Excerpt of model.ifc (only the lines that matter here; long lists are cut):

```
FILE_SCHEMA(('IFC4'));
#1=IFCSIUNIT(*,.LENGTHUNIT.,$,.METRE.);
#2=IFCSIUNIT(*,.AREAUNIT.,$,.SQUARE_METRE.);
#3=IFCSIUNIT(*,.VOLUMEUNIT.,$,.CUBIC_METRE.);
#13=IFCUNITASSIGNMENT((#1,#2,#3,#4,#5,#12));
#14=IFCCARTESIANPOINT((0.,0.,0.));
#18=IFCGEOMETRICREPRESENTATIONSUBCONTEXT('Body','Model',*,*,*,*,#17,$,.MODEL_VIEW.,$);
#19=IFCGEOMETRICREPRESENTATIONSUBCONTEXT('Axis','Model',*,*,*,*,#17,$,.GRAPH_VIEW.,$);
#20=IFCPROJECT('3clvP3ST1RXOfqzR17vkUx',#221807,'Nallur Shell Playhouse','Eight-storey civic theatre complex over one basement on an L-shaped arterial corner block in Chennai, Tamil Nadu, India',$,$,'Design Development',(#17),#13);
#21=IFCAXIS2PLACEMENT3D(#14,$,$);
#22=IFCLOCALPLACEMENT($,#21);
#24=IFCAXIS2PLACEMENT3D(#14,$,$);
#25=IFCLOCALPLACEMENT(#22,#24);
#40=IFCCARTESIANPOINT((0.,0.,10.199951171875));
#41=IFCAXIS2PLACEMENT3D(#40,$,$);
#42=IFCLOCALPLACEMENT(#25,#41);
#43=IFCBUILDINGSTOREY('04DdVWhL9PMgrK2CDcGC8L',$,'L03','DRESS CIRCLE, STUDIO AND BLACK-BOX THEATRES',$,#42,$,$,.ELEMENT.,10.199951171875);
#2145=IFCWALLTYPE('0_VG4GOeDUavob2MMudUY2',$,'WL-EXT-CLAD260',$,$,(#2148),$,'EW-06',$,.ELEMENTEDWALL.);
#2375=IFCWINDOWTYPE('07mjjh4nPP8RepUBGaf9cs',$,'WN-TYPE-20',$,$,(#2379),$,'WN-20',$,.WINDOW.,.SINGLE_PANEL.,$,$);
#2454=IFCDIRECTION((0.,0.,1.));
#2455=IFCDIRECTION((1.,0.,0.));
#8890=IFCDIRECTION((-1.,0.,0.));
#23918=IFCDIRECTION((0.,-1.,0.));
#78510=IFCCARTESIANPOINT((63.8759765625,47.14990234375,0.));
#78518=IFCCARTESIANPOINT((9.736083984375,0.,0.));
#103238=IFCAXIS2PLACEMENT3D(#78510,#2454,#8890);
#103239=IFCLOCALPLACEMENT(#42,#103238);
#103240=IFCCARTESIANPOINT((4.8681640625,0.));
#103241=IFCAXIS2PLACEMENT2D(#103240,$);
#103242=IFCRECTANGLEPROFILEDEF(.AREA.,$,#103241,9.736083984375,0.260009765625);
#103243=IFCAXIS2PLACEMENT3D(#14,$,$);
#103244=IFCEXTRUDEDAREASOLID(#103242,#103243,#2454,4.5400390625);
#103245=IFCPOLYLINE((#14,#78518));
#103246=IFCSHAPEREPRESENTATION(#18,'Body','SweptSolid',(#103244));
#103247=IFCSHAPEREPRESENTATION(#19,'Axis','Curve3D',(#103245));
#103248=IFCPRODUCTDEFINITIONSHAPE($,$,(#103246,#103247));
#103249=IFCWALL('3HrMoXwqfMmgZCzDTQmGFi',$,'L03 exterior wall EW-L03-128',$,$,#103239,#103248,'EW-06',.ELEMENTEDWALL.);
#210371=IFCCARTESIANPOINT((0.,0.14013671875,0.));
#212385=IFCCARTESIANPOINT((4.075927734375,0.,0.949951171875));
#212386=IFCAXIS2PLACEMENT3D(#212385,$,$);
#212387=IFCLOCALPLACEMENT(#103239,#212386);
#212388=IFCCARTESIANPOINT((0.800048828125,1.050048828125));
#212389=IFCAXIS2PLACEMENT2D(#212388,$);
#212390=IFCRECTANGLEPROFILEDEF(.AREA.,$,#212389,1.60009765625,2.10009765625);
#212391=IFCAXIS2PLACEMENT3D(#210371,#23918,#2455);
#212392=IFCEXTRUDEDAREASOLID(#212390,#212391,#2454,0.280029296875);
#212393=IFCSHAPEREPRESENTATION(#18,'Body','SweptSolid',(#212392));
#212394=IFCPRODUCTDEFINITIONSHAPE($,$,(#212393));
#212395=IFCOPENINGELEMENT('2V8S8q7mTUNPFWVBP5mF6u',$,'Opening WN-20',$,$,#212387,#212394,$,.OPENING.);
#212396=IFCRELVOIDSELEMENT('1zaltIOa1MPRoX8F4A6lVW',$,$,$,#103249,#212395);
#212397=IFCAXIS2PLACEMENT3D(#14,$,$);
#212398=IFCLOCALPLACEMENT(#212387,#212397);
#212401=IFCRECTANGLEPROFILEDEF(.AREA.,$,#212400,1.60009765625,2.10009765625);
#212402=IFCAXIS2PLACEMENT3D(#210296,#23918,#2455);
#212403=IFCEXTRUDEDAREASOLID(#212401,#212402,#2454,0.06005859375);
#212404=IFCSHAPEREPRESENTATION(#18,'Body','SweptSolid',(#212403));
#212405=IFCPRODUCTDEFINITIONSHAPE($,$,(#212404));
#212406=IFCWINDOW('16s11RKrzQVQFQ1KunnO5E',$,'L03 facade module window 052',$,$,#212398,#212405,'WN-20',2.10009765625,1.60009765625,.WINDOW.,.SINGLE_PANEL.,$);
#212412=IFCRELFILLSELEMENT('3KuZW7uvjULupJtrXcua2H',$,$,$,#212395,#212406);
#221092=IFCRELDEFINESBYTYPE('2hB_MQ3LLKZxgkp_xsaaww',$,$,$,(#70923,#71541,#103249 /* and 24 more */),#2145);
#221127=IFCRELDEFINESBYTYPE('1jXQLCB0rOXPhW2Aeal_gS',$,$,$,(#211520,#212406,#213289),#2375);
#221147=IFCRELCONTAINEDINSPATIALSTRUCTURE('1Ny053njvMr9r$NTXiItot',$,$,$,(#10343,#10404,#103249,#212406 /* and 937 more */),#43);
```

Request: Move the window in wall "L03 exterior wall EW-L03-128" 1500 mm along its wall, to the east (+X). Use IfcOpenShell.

```python
import ifcopenshell
import ifcopenshell.api.geometry
import ifcopenshell.util.placement
import ifcopenshell.util.unit

model = ifcopenshell.open("model.ifc")
unit_scale = ifcopenshell.util.unit.calculate_unit_scale(model)

window = model.by_guid("16s11RKrzQVQFQ1KunnO5E")
opening = window.FillsVoids[0].RelatingOpeningElement
wall = opening.VoidsElements[0].RelatingBuildingElement

wall_matrix = ifcopenshell.util.placement.get_local_placement(wall.ObjectPlacement)
shift = wall_matrix[:3, 0] * -1.5 / unit_scale
before = ifcopenshell.util.placement.get_local_placement(window.ObjectPlacement)[:3, 3].copy()

# The window is placed relative to its opening, so it follows when the opening moves.
matrix = ifcopenshell.util.placement.get_local_placement(opening.ObjectPlacement)
matrix[:3, 3] += shift
ifcopenshell.api.geometry.edit_object_placement(
    model, product=opening, matrix=matrix, is_si=False, should_transform_children=True
)

after = ifcopenshell.util.placement.get_local_placement(window.ObjectPlacement)[:3, 3]
print("window moved by", (after - before).round(3) + 0.0)

model.write("model_edited.ifc")
```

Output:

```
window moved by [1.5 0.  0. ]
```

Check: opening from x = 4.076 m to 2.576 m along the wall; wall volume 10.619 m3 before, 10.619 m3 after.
